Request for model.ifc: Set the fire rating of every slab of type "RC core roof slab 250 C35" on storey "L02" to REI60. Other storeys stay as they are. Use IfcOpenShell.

First a look at what the model holds.

```python
import ifcopenshell
import ifcopenshell.util.element

model = ifcopenshell.open("model.ifc")
print(model.schema)
storey = next(s for s in model.by_type("IfcBuildingStorey") if s.Name == "L02")
slabs = [e for e in ifcopenshell.util.element.get_decomposition(storey) if e.is_a("IfcSlab")]
seen = {}
for e in slabs:
    element_type = ifcopenshell.util.element.get_type(e)
    key = (element_type.Name if element_type != e and element_type else None, ifcopenshell.util.element.get_pset(e, "Pset_SlabCommon", "FireRating"))
    seen[key] = seen.get(key, 0) + 1
for (name, value), count in sorted(seen.items(), key=str):
    print(count, "x", name, "|", value)
```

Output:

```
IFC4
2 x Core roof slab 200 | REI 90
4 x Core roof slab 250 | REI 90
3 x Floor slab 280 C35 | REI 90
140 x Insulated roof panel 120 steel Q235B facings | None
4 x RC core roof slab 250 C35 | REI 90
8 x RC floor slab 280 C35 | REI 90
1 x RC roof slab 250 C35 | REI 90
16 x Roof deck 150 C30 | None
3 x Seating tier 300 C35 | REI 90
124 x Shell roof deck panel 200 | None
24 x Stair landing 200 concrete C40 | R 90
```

```python
import ifcopenshell
import ifcopenshell.api.pset
import ifcopenshell.util.element

model = ifcopenshell.open("model.ifc")

storey = next(s for s in model.by_type("IfcBuildingStorey") if s.Name == "L02")
slabs = [e for e in ifcopenshell.util.element.get_decomposition(storey) if e.is_a("IfcSlab")]

count = 0
for e in slabs:
    element_type = ifcopenshell.util.element.get_type(e)
    if element_type in (None, e) or element_type.Name != "RC core roof slab 250 C35":
        continue
    # add_pset returns the element's existing set when there is one.
    pset = ifcopenshell.api.pset.add_pset(model, product=e, name="Pset_SlabCommon")
    ifcopenshell.api.pset.edit_pset(model, pset=pset, properties={"FireRating": "REI60"})
    count += 1

print(count, "slabs updated")

model.write("model_edited.ifc")
```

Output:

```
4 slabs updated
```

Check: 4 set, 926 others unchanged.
